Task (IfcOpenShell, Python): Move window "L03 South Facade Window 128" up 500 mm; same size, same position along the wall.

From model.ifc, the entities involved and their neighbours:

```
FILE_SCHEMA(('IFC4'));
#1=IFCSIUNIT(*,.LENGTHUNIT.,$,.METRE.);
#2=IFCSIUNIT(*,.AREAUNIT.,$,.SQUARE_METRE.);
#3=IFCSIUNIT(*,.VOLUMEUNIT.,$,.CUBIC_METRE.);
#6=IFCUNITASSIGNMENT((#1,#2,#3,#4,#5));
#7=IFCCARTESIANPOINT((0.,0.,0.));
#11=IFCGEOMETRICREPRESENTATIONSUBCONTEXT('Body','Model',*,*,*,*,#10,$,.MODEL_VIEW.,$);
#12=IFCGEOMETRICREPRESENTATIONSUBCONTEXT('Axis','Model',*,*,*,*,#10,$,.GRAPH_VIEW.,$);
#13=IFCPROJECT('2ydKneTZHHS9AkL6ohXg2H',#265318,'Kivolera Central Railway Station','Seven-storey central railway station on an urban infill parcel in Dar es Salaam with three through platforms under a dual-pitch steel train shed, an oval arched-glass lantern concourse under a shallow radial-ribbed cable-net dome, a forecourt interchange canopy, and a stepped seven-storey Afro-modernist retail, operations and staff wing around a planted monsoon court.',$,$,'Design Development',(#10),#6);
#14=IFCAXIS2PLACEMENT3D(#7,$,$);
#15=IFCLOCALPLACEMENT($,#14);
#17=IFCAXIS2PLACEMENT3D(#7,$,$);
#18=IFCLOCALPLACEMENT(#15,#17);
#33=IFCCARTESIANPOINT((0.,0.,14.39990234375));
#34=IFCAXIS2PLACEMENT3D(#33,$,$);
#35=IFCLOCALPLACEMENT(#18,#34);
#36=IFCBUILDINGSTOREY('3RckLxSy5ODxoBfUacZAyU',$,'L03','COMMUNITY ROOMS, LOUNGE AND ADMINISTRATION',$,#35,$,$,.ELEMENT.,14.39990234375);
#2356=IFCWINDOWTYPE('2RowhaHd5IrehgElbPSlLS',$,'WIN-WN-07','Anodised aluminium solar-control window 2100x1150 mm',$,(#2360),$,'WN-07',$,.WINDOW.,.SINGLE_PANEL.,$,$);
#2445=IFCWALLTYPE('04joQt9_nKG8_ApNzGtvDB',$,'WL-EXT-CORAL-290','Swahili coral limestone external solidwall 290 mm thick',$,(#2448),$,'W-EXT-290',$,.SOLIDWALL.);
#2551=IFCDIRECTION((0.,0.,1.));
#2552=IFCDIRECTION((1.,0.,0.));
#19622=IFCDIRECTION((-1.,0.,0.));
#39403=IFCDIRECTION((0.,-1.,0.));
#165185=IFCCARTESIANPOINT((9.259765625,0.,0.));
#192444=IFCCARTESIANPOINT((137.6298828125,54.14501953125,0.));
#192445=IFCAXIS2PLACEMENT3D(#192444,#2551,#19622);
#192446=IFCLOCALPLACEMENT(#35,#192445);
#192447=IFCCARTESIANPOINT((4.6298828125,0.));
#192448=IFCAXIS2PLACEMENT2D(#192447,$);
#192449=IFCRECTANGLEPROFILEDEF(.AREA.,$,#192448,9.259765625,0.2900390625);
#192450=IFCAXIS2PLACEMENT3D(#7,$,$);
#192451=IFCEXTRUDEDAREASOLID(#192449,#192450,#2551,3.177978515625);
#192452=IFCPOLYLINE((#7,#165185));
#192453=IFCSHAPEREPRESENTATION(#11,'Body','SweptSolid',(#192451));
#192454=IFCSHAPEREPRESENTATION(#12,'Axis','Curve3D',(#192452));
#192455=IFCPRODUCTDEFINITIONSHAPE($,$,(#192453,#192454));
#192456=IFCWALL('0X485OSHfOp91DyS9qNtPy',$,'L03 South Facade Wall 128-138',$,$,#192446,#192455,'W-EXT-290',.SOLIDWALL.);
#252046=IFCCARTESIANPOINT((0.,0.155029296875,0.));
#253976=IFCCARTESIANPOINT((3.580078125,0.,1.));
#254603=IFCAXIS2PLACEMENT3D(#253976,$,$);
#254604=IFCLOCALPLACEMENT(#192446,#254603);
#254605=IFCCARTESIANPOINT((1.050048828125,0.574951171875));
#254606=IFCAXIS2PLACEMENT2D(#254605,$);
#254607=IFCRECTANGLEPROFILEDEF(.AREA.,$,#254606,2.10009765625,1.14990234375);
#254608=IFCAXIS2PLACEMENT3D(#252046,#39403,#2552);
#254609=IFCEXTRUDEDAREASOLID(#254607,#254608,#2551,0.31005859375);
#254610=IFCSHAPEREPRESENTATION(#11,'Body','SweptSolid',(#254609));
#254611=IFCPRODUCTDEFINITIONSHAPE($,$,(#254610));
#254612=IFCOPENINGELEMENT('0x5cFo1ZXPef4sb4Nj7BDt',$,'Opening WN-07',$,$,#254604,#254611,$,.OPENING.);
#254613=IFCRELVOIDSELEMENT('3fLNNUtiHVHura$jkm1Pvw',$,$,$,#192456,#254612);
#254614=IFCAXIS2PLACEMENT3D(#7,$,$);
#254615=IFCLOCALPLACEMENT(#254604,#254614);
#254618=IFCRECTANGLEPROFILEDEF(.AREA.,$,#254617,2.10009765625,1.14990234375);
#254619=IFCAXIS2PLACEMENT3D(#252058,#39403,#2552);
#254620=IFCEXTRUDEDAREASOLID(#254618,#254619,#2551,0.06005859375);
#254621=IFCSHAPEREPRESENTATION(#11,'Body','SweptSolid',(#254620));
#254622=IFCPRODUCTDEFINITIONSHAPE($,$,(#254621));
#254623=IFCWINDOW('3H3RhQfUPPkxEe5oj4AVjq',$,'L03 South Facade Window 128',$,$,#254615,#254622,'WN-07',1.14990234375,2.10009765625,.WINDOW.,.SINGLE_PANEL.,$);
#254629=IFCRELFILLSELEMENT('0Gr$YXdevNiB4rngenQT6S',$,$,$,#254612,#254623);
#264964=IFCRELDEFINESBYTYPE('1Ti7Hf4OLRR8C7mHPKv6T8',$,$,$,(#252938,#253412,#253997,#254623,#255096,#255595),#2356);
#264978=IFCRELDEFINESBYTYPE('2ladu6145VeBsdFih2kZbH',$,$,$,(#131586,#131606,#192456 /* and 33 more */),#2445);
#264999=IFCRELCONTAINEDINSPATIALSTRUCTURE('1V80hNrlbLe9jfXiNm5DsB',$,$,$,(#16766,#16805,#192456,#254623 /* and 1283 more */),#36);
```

```python
import numpy as np
import ifcopenshell
import ifcopenshell.api.geometry
import ifcopenshell.util.placement
import ifcopenshell.util.unit

model = ifcopenshell.open("model.ifc")
unit_scale = ifcopenshell.util.unit.calculate_unit_scale(model)

window = model.by_guid("3H3RhQfUPPkxEe5oj4AVjq")
opening = window.FillsVoids[0].RelatingOpeningElement
dz = 0.5 / unit_scale

shift = np.array([0.0, 0.0, dz])
# The window is placed relative to its opening, so it follows when the opening moves.
matrix = ifcopenshell.util.placement.get_local_placement(opening.ObjectPlacement)
matrix[:3, 3] += shift
ifcopenshell.api.geometry.edit_object_placement(
    model, product=opening, matrix=matrix, is_si=False, should_transform_children=True
)

print(f"moved by {dz * unit_scale:+.3f} m")

model.write("model-out.ifc")
```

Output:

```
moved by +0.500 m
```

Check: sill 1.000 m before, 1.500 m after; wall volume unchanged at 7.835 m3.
